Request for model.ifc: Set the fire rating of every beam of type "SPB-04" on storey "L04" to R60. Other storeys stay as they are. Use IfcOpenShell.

First a look at what the model holds.

```python
import ifcopenshell
import ifcopenshell.util.element

model = ifcopenshell.open("model.ifc")
print(model.schema)
storey = next(s for s in model.by_type("IfcBuildingStorey") if s.Name == "L04")
beams = [e for e in ifcopenshell.util.element.get_decomposition(storey) if e.is_a("IfcBeam")]
seen = {}
for e in beams:
    element_type = ifcopenshell.util.element.get_type(e)
    key = (element_type.Name if element_type != e and element_type else None, ifcopenshell.util.element.get_pset(e, "Pset_BeamCommon", "FireRating"))
    seen[key] = seen.get(key, 0) + 1
for (name, value), count in sorted(seen.items(), key=str):
    print(count, "x", name, "|", value)
```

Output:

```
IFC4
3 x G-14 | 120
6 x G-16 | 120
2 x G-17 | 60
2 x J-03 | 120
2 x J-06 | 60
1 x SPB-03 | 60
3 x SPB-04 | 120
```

```python
import ifcopenshell
import ifcopenshell.api.pset
import ifcopenshell.util.element

model = ifcopenshell.open("model.ifc")

storey = next(s for s in model.by_type("IfcBuildingStorey") if s.Name == "L04")
beams = [e for e in ifcopenshell.util.element.get_decomposition(storey) if e.is_a("IfcBeam")]

count = 0
for e in beams:
    element_type = ifcopenshell.util.element.get_type(e)
    if element_type in (None, e) or element_type.Name != "SPB-04":
        continue
    # add_pset returns the element's existing set when there is one.
    pset = ifcopenshell.api.pset.add_pset(model, product=e, name="Pset_BeamCommon")
    ifcopenshell.api.pset.edit_pset(model, pset=pset, properties={"FireRating": "R60"})
    count += 1

print(count, "beams updated")

model.write("model_rev.ifc")
```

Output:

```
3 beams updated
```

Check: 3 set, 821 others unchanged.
